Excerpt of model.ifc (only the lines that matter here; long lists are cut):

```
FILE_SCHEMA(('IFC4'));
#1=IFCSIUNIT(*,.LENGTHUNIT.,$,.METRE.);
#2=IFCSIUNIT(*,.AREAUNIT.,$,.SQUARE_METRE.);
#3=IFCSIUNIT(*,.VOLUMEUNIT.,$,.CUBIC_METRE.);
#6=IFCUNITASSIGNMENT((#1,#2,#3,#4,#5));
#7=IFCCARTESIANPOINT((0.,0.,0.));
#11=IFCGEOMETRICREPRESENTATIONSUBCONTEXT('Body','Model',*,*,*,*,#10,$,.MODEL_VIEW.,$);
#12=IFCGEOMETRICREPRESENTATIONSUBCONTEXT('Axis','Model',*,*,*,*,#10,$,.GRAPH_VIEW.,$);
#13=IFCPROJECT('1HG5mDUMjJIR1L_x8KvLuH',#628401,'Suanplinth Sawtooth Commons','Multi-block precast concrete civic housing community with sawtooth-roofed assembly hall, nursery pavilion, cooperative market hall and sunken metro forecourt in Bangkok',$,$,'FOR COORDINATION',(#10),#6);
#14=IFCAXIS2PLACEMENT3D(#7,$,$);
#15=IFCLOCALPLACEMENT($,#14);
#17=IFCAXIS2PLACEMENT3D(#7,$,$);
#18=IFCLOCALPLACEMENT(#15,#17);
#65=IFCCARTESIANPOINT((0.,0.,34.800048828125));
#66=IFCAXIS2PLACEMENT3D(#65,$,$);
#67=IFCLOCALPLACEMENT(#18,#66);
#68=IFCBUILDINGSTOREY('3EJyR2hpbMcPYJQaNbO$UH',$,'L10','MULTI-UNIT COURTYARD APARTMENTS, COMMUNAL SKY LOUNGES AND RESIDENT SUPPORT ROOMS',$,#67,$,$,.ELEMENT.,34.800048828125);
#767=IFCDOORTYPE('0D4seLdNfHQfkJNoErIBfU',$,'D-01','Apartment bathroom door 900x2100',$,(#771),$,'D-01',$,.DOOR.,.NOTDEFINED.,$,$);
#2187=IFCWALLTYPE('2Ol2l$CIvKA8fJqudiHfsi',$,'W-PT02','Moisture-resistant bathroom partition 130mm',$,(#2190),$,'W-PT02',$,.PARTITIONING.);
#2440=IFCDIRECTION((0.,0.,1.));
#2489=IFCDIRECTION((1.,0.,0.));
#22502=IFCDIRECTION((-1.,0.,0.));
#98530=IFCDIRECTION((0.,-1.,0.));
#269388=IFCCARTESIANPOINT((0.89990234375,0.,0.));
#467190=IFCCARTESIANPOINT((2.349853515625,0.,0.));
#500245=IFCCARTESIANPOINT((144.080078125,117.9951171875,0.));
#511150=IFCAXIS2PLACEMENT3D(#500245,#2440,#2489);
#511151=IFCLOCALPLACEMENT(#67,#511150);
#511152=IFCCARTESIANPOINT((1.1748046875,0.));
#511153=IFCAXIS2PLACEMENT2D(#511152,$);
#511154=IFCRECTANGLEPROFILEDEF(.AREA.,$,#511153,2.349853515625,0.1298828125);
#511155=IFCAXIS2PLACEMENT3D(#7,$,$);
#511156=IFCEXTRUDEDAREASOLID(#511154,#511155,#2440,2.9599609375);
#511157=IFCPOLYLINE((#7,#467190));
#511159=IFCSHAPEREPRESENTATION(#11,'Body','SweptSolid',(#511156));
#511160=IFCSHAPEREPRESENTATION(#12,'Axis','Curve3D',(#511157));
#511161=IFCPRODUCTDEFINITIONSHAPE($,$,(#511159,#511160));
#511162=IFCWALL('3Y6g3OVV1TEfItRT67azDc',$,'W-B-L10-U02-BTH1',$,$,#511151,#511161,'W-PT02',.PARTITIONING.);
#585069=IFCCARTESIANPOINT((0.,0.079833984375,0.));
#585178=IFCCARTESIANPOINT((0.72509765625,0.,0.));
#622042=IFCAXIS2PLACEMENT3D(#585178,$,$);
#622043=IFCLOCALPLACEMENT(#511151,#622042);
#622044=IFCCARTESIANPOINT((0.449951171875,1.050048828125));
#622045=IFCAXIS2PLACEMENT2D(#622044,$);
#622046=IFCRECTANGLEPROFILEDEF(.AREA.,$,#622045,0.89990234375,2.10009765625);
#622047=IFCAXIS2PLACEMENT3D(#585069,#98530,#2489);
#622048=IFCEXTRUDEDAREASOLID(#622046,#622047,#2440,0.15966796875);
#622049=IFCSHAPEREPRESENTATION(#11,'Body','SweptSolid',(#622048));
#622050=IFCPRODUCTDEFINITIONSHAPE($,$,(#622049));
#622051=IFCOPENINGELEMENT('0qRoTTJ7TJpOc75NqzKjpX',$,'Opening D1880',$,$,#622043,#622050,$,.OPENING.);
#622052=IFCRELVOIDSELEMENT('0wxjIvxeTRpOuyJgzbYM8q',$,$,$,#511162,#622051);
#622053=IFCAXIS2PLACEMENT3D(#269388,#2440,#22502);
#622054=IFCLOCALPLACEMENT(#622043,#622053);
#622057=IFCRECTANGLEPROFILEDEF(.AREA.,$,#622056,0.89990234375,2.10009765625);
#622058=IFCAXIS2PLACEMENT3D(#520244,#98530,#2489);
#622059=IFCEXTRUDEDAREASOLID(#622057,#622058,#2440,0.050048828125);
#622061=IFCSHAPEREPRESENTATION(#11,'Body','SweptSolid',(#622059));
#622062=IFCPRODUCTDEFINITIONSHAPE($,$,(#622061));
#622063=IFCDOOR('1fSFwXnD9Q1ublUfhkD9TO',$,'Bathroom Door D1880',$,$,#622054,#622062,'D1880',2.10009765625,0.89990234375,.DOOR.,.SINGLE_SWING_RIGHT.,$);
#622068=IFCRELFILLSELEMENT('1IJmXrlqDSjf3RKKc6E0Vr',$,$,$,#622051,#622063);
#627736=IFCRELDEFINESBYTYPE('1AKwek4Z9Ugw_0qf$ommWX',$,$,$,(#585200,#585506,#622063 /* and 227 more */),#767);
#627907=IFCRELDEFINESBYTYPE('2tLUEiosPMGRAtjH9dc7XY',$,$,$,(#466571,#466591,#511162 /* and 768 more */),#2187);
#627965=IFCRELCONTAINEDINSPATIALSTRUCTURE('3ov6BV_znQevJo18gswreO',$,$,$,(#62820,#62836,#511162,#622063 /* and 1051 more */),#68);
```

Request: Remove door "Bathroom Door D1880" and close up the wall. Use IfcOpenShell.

```python
import ifcopenshell
import ifcopenshell.api.feature
import ifcopenshell.api.root
import ifcopenshell.geom
import ifcopenshell.util.shape

model = ifcopenshell.open("model.ifc")
settings = ifcopenshell.geom.settings()


def volume(element):
    """Net volume in cubic metres, openings subtracted."""
    shape = ifcopenshell.geom.create_shape(settings, element)
    return ifcopenshell.util.shape.get_volume(shape.geometry)


door = model.by_guid("1fSFwXnD9Q1ublUfhkD9TO")
opening = door.FillsVoids[0].RelatingOpeningElement
wall = opening.VoidsElements[0].RelatingBuildingElement
before = volume(wall)

ifcopenshell.api.root.remove_product(model, product=door)
ifcopenshell.api.feature.remove_feature(model, feature=opening)

after = volume(wall)

print(f"wall volume {before:.3f} -> {after:.3f} m3")

model.write("model-out.ifc")
```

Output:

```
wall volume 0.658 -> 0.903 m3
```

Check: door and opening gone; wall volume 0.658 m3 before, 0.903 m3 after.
